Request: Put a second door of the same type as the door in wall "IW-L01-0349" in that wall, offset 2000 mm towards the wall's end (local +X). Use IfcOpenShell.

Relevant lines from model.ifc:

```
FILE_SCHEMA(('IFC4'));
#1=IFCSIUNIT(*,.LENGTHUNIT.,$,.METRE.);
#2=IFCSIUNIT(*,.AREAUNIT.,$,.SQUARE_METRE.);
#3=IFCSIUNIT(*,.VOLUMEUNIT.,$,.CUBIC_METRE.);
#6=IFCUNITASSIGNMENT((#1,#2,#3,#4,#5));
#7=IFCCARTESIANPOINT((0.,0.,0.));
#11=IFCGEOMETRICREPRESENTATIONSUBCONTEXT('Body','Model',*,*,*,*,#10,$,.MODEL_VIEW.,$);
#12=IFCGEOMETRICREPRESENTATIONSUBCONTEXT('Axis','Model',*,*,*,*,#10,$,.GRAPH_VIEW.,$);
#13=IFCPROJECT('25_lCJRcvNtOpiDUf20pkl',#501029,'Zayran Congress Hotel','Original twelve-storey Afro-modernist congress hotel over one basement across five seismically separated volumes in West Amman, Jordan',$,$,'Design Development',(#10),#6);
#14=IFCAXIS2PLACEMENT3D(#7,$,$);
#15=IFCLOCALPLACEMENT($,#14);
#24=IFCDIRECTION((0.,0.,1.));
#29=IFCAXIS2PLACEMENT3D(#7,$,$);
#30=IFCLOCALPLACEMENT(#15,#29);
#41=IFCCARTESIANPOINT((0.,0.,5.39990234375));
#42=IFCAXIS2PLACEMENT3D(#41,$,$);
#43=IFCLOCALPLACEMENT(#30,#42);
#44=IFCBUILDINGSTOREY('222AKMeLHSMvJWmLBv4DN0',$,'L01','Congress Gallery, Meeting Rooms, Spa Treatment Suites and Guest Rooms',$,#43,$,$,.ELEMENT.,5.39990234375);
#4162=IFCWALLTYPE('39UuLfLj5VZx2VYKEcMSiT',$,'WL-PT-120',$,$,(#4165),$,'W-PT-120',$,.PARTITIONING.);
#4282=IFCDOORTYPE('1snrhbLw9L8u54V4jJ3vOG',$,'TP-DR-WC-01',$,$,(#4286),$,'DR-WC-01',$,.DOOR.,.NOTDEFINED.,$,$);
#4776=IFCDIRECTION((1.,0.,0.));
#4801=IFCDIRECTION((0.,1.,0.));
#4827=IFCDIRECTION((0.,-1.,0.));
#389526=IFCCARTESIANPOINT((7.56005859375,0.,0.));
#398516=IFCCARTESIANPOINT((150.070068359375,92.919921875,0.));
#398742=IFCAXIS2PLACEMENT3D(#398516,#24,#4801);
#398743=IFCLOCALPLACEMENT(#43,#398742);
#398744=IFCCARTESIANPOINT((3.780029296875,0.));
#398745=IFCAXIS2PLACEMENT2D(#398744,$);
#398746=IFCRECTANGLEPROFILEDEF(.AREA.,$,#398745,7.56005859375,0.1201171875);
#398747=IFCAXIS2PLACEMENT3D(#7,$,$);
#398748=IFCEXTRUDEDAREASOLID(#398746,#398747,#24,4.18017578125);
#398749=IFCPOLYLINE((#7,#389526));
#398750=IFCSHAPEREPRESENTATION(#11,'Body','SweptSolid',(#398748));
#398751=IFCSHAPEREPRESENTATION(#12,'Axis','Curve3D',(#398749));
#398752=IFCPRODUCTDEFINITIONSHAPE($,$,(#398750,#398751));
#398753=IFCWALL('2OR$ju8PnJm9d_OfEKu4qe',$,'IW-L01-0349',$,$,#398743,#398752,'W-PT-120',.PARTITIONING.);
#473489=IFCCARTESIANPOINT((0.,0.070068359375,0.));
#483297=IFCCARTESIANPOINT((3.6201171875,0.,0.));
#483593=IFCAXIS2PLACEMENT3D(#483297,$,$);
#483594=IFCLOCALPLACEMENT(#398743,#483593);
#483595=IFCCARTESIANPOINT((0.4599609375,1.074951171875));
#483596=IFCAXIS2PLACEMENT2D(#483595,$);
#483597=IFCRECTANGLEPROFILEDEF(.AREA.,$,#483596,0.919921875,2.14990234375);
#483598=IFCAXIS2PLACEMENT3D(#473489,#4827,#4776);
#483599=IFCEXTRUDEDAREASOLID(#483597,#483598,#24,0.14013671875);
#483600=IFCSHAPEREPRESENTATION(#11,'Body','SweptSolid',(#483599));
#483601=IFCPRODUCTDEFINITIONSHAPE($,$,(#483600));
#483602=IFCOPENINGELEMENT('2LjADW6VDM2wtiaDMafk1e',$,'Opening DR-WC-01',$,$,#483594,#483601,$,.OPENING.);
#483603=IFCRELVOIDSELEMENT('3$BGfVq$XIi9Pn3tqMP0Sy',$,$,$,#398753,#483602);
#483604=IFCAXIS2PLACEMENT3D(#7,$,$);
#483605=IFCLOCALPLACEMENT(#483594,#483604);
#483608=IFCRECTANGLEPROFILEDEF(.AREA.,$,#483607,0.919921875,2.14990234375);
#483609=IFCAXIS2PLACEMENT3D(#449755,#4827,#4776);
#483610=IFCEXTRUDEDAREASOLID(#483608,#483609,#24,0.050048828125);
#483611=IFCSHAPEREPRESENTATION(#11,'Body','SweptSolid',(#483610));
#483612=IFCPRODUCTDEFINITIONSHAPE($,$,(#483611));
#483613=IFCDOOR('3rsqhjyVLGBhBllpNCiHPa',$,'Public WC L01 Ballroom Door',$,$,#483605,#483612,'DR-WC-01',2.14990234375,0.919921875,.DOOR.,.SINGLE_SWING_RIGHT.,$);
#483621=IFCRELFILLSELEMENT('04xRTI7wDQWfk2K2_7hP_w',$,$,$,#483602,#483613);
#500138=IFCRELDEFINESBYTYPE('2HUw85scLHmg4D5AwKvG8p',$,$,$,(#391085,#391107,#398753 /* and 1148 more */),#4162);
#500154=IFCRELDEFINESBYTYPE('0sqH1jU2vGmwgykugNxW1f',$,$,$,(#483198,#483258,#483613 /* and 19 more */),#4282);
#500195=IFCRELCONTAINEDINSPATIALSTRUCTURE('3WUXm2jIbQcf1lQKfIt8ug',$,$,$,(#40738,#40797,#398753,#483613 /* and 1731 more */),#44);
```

```python
import ifcopenshell
import ifcopenshell.api.feature
import ifcopenshell.api.geometry
import ifcopenshell.api.root
import ifcopenshell.geom
import ifcopenshell.util.element
import ifcopenshell.util.placement
import ifcopenshell.util.shape
import ifcopenshell.util.unit

model = ifcopenshell.open("model.ifc")
unit_scale = ifcopenshell.util.unit.calculate_unit_scale(model)
settings = ifcopenshell.geom.settings()


def volume(element):
    """Net volume in cubic metres, openings subtracted."""
    shape = ifcopenshell.geom.create_shape(settings, element)
    return ifcopenshell.util.shape.get_volume(shape.geometry)


door = model.by_guid("3rsqhjyVLGBhBllpNCiHPa")
opening = door.FillsVoids[0].RelatingOpeningElement
wall = opening.VoidsElements[0].RelatingBuildingElement
before = volume(wall)
shift = ifcopenshell.util.placement.get_local_placement(wall.ObjectPlacement)[:3, 0] * 2 / unit_scale

# copy_class copies the void relationship, type, container and properties, but no geometry.
new_opening = ifcopenshell.api.root.copy_class(model, product=opening)
new_opening.Representation = ifcopenshell.util.element.copy_deep(
    model, opening.Representation, exclude=["IfcGeometricRepresentationContext", "IfcRepresentationMap"]
)
new_door = ifcopenshell.api.root.copy_class(model, product=door)
new_door.Representation = ifcopenshell.util.element.copy_deep(
    model, door.Representation, exclude=["IfcGeometricRepresentationContext", "IfcRepresentationMap"]
)
new_door.Tag = None
ifcopenshell.api.feature.add_filling(model, opening=new_opening, element=new_door)

for old, new in ((opening, new_opening), (door, new_door)):
    matrix = ifcopenshell.util.placement.get_local_placement(old.ObjectPlacement)
    matrix[:3, 3] += shift
    ifcopenshell.api.geometry.edit_object_placement(model, product=new, matrix=matrix, is_si=False)

after = volume(wall)

print(f"wall volume {before:.3f} -> {after:.3f} m3")

model.write("model_updated.ifc")
```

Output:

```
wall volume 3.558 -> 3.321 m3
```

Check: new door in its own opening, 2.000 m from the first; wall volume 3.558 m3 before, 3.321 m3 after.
